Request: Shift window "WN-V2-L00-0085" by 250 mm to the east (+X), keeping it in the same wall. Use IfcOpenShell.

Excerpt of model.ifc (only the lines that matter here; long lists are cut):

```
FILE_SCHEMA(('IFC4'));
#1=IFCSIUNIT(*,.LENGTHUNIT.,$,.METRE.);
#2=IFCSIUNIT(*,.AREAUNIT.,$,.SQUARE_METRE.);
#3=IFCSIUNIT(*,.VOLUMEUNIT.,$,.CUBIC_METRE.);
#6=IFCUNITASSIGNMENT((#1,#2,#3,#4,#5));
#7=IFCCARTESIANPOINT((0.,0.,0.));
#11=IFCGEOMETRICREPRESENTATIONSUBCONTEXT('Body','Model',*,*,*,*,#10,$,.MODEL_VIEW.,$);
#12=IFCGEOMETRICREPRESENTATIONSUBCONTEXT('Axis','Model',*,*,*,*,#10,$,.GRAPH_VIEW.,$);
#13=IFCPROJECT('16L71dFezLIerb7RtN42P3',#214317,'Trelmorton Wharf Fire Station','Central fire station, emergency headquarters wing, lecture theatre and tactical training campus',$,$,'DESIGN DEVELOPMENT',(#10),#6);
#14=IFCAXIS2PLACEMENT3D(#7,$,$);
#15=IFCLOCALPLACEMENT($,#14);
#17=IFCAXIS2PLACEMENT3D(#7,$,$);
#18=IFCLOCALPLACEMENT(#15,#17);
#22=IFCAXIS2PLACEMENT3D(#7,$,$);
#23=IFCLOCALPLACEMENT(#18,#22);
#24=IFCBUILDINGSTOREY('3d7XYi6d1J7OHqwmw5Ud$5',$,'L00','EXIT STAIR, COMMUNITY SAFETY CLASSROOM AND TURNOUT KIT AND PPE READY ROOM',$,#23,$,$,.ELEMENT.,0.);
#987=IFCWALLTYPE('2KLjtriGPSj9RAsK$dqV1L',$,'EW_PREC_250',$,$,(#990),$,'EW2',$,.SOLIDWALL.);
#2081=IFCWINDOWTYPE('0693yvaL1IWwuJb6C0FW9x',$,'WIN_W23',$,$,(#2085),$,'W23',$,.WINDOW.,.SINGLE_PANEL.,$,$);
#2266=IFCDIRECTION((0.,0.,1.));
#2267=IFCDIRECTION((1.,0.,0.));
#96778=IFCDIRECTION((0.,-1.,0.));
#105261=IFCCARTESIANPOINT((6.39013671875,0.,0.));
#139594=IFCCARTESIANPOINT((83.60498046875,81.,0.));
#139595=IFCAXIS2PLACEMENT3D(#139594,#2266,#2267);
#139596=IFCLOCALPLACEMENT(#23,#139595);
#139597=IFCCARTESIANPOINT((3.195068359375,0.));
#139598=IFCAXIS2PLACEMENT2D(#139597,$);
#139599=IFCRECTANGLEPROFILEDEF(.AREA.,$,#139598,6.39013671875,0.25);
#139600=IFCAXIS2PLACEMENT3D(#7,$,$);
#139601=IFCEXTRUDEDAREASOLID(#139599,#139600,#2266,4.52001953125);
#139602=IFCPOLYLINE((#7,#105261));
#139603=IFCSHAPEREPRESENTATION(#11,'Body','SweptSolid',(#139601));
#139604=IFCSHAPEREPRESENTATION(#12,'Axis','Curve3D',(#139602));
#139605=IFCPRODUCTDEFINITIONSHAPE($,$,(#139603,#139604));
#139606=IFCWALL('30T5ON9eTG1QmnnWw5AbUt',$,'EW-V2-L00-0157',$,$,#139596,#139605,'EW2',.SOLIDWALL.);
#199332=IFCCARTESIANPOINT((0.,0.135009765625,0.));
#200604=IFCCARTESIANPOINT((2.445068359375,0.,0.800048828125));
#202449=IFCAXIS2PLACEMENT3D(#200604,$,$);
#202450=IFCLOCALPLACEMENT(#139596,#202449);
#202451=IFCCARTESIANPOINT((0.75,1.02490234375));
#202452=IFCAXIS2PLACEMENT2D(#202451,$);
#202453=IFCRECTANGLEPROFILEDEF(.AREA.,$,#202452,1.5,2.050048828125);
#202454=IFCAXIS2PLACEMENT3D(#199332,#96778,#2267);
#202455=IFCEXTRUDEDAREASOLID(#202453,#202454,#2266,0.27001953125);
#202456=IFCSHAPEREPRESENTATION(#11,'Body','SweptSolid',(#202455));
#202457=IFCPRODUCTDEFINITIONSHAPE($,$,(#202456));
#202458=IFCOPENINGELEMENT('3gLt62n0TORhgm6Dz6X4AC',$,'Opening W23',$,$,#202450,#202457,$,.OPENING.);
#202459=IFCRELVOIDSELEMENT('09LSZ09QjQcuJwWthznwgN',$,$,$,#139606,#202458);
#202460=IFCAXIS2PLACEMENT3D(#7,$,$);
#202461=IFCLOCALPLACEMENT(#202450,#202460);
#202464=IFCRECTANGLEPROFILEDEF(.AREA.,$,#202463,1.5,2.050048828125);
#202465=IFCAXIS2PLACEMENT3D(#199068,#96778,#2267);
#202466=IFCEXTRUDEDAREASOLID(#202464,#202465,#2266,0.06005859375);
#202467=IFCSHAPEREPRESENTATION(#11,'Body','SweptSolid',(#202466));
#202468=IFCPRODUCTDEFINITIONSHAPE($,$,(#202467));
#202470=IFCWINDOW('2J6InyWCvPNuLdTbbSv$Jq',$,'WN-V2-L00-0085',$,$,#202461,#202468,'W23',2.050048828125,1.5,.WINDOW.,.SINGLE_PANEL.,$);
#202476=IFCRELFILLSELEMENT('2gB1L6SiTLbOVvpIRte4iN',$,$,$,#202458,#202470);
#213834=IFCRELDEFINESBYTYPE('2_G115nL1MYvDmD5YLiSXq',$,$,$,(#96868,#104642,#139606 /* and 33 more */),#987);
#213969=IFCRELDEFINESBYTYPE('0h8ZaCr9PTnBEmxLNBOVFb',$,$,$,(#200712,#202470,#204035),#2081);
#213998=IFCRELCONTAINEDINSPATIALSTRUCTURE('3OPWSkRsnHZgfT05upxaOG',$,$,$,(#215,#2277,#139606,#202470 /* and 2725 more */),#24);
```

```python
import ifcopenshell
import ifcopenshell.api.geometry
import ifcopenshell.util.placement
import ifcopenshell.util.unit

model = ifcopenshell.open("model.ifc")
unit_scale = ifcopenshell.util.unit.calculate_unit_scale(model)

window = model.by_guid("2J6InyWCvPNuLdTbbSv$Jq")
opening = window.FillsVoids[0].RelatingOpeningElement
wall = opening.VoidsElements[0].RelatingBuildingElement

wall_matrix = ifcopenshell.util.placement.get_local_placement(wall.ObjectPlacement)
shift = wall_matrix[:3, 0] * 0.25 / unit_scale
before = ifcopenshell.util.placement.get_local_placement(window.ObjectPlacement)[:3, 3].copy()

# The window is placed relative to its opening, so it follows when the opening moves.
matrix = ifcopenshell.util.placement.get_local_placement(opening.ObjectPlacement)
matrix[:3, 3] += shift
ifcopenshell.api.geometry.edit_object_placement(
    model, product=opening, matrix=matrix, is_si=False, should_transform_children=True
)

after = ifcopenshell.util.placement.get_local_placement(window.ObjectPlacement)[:3, 3]
print("window moved by", (after - before).round(3) + 0.0)

model.write("model-out.ifc")
```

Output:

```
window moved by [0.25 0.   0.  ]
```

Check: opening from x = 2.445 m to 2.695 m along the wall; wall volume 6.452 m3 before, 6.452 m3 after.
